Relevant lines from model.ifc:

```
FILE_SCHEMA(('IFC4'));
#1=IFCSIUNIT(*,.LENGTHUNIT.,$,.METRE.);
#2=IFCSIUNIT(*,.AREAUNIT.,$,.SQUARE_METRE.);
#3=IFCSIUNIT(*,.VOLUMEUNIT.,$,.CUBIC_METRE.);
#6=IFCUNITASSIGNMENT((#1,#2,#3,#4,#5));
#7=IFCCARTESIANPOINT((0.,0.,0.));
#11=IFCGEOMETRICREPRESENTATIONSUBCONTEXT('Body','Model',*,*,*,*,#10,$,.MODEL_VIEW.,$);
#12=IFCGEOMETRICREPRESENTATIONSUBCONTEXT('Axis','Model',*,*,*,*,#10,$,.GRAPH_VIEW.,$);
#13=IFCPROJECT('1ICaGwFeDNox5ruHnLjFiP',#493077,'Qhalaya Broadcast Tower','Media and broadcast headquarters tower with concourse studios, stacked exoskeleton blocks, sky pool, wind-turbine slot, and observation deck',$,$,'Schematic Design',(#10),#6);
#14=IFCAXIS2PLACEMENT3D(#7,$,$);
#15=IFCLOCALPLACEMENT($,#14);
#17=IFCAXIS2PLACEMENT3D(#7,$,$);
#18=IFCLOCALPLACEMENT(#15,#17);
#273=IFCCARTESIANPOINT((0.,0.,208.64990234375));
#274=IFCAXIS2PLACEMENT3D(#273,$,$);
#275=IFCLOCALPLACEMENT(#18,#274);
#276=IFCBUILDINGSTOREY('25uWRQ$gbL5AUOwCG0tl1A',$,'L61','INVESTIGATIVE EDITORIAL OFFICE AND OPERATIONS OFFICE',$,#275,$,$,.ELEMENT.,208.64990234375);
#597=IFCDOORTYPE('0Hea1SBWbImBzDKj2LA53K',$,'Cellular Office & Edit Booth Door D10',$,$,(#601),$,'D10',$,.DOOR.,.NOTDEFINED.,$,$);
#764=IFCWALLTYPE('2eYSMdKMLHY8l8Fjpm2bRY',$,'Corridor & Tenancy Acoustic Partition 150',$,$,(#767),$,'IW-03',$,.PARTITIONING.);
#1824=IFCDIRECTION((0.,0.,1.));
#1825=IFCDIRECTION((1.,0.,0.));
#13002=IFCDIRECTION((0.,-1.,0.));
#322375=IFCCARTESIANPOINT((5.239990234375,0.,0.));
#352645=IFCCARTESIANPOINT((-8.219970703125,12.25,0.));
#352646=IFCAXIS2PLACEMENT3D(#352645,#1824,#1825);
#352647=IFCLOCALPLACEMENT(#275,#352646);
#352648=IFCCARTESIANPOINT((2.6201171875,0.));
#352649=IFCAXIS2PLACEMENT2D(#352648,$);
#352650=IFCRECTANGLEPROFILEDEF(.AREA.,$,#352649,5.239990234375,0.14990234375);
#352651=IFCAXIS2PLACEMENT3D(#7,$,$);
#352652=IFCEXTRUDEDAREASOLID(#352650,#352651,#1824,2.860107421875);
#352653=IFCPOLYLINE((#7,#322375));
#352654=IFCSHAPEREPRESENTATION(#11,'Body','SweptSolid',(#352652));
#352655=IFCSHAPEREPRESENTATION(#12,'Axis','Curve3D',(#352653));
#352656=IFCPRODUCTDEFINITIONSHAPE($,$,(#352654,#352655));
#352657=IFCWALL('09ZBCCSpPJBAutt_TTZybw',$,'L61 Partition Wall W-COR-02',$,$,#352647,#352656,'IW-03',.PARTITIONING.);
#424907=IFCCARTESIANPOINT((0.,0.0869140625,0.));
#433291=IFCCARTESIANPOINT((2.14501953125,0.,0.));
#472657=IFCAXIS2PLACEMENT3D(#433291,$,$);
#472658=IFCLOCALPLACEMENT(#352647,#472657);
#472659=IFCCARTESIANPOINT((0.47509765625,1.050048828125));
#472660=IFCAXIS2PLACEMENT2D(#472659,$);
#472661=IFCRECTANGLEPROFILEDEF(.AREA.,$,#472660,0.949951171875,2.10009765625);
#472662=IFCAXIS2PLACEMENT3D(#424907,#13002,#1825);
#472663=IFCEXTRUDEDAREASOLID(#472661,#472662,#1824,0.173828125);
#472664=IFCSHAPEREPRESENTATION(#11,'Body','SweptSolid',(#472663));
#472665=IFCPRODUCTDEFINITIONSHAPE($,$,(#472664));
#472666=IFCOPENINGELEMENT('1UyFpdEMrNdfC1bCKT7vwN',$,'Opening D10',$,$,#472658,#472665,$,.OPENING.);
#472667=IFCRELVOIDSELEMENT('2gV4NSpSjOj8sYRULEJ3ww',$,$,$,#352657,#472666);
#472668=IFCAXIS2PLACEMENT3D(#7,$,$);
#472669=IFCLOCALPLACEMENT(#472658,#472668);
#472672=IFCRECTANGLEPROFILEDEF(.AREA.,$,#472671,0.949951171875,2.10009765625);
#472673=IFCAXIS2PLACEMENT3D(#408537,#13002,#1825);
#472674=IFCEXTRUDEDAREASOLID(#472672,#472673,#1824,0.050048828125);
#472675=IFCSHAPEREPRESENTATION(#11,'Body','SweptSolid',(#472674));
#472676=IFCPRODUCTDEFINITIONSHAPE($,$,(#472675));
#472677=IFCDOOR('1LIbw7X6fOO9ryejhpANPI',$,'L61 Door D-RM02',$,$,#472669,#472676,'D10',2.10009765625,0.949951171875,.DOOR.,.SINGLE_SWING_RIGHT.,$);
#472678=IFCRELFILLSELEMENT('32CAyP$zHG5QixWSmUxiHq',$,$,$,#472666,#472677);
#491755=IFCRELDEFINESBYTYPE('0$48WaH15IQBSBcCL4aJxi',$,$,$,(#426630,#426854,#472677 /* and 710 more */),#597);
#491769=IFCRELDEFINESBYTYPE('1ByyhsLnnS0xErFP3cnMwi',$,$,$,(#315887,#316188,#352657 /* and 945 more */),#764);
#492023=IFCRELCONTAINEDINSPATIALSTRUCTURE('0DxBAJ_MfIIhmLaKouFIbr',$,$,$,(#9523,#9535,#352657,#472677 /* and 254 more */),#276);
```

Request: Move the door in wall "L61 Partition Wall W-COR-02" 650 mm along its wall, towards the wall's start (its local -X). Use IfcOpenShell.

```python
import ifcopenshell
import ifcopenshell.api.geometry
import ifcopenshell.util.placement
import ifcopenshell.util.unit

model = ifcopenshell.open("model.ifc")
unit_scale = ifcopenshell.util.unit.calculate_unit_scale(model)

door = model.by_guid("1LIbw7X6fOO9ryejhpANPI")
opening = door.FillsVoids[0].RelatingOpeningElement
wall = opening.VoidsElements[0].RelatingBuildingElement

wall_matrix = ifcopenshell.util.placement.get_local_placement(wall.ObjectPlacement)
shift = wall_matrix[:3, 0] * -0.65 / unit_scale
before = ifcopenshell.util.placement.get_local_placement(door.ObjectPlacement)[:3, 3].copy()

# The door is placed relative to its opening, so it follows when the opening moves.
matrix = ifcopenshell.util.placement.get_local_placement(opening.ObjectPlacement)
matrix[:3, 3] += shift
ifcopenshell.api.geometry.edit_object_placement(
    model, product=opening, matrix=matrix, is_si=False, should_transform_children=True
)

after = ifcopenshell.util.placement.get_local_placement(door.ObjectPlacement)[:3, 3]
print("door moved by", (after - before).round(3) + 0.0)

model.write("model_rev.ifc")
```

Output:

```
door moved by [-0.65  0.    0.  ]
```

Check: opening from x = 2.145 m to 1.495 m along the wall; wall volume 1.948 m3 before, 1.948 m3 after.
